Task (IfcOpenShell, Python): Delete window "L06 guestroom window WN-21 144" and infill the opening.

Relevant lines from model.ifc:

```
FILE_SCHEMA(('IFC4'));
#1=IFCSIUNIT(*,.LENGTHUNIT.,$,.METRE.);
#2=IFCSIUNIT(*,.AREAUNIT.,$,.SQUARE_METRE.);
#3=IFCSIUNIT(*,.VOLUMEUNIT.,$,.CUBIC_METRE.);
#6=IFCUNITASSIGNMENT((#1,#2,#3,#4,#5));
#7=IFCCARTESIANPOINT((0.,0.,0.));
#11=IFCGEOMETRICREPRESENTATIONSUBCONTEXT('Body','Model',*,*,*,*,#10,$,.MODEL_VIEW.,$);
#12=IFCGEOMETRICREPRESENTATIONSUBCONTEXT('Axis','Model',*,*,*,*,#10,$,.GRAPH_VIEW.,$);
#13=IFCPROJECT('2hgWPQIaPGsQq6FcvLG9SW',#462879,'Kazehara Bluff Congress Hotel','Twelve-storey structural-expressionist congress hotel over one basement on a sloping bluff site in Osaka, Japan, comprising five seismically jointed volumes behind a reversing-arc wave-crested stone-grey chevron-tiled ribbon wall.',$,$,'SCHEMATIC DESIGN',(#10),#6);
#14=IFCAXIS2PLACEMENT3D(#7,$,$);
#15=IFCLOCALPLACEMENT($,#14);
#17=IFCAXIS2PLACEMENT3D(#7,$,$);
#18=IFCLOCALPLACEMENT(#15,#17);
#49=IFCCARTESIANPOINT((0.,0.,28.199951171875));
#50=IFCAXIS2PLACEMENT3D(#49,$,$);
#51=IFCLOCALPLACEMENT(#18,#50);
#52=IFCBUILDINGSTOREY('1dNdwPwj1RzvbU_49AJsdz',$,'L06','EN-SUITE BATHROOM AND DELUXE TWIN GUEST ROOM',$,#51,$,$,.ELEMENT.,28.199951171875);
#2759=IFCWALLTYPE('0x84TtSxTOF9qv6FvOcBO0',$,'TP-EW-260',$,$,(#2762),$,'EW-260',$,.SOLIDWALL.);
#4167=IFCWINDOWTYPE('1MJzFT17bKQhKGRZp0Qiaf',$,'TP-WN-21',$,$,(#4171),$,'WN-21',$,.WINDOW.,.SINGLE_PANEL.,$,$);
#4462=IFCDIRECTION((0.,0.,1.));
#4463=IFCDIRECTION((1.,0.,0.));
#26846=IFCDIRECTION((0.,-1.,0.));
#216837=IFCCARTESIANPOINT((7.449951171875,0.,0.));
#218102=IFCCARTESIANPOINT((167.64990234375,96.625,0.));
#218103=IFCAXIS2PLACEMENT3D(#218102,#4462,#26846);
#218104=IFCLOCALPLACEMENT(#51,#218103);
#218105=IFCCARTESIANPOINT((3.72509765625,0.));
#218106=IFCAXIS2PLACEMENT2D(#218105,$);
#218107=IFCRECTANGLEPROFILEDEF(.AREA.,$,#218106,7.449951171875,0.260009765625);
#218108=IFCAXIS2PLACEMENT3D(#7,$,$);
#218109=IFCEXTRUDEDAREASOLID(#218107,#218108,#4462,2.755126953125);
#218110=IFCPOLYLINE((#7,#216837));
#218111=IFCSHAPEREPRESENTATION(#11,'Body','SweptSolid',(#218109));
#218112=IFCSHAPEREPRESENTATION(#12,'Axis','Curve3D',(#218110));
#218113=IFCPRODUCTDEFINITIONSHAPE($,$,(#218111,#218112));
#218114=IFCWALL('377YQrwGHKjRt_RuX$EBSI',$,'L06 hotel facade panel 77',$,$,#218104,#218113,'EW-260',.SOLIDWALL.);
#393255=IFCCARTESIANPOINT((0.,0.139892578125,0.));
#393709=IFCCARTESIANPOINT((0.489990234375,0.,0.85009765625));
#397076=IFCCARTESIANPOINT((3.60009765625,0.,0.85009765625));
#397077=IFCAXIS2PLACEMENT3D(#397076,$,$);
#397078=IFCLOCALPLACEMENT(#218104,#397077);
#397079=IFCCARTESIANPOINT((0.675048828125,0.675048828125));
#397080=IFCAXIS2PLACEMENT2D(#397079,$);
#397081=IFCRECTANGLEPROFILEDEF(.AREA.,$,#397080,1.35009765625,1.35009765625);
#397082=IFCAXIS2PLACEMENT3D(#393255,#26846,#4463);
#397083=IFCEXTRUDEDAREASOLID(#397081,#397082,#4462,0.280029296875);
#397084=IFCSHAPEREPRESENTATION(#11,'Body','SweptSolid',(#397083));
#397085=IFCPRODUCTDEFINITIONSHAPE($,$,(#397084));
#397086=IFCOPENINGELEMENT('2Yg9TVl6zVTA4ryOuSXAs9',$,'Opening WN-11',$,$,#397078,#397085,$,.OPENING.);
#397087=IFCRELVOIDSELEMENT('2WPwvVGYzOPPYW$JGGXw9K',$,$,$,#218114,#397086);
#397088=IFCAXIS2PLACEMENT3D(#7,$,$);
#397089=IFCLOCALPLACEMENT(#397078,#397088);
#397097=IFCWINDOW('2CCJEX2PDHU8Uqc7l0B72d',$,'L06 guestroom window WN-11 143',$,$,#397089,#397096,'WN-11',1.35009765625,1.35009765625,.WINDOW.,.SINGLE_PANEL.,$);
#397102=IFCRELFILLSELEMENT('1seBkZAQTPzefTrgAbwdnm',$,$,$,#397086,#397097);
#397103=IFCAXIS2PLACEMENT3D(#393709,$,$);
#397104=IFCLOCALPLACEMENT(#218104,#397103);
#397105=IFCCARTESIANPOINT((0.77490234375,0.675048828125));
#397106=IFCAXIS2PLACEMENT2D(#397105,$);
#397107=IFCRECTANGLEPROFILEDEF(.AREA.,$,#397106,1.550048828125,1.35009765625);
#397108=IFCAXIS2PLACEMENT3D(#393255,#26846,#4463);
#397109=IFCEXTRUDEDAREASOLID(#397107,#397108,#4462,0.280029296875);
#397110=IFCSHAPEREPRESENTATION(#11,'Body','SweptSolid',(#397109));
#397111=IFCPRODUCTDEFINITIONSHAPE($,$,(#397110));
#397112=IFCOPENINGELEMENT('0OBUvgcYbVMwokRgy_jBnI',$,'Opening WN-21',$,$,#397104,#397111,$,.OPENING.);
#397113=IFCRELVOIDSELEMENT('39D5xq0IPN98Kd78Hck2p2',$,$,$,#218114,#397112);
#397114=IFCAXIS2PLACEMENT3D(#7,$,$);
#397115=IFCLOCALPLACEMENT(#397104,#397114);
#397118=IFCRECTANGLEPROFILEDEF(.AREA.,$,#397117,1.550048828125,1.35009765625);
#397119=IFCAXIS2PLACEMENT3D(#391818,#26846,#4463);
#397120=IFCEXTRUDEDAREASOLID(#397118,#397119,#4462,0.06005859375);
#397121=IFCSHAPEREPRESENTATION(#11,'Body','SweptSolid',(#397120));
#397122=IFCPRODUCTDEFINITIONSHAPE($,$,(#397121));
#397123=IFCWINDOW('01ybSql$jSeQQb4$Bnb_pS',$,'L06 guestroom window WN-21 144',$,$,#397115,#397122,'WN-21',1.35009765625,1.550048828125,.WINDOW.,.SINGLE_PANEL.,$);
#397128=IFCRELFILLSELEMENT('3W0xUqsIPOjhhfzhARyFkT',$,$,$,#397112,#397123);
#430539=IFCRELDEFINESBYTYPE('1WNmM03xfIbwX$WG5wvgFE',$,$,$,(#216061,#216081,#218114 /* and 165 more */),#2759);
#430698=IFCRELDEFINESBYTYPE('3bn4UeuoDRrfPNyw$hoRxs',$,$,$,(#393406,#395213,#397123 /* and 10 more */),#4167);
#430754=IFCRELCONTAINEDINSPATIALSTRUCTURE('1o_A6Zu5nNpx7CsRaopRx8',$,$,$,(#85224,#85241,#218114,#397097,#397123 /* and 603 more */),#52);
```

```python
import ifcopenshell
import ifcopenshell.api.feature
import ifcopenshell.api.root
import ifcopenshell.geom
import ifcopenshell.util.shape

model = ifcopenshell.open("model.ifc")
settings = ifcopenshell.geom.settings()


def volume(element):
    """Net volume in cubic metres, openings subtracted."""
    shape = ifcopenshell.geom.create_shape(settings, element)
    return ifcopenshell.util.shape.get_volume(shape.geometry)


window = model.by_guid("01ybSql$jSeQQb4$Bnb_pS")
opening = window.FillsVoids[0].RelatingOpeningElement
wall = opening.VoidsElements[0].RelatingBuildingElement
before = volume(wall)

ifcopenshell.api.root.remove_product(model, product=window)
ifcopenshell.api.feature.remove_feature(model, feature=opening)

after = volume(wall)

print(f"wall volume {before:.3f} -> {after:.3f} m3")

model.write("model_updated.ifc")
```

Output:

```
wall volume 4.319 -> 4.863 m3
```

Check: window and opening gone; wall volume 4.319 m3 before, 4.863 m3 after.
